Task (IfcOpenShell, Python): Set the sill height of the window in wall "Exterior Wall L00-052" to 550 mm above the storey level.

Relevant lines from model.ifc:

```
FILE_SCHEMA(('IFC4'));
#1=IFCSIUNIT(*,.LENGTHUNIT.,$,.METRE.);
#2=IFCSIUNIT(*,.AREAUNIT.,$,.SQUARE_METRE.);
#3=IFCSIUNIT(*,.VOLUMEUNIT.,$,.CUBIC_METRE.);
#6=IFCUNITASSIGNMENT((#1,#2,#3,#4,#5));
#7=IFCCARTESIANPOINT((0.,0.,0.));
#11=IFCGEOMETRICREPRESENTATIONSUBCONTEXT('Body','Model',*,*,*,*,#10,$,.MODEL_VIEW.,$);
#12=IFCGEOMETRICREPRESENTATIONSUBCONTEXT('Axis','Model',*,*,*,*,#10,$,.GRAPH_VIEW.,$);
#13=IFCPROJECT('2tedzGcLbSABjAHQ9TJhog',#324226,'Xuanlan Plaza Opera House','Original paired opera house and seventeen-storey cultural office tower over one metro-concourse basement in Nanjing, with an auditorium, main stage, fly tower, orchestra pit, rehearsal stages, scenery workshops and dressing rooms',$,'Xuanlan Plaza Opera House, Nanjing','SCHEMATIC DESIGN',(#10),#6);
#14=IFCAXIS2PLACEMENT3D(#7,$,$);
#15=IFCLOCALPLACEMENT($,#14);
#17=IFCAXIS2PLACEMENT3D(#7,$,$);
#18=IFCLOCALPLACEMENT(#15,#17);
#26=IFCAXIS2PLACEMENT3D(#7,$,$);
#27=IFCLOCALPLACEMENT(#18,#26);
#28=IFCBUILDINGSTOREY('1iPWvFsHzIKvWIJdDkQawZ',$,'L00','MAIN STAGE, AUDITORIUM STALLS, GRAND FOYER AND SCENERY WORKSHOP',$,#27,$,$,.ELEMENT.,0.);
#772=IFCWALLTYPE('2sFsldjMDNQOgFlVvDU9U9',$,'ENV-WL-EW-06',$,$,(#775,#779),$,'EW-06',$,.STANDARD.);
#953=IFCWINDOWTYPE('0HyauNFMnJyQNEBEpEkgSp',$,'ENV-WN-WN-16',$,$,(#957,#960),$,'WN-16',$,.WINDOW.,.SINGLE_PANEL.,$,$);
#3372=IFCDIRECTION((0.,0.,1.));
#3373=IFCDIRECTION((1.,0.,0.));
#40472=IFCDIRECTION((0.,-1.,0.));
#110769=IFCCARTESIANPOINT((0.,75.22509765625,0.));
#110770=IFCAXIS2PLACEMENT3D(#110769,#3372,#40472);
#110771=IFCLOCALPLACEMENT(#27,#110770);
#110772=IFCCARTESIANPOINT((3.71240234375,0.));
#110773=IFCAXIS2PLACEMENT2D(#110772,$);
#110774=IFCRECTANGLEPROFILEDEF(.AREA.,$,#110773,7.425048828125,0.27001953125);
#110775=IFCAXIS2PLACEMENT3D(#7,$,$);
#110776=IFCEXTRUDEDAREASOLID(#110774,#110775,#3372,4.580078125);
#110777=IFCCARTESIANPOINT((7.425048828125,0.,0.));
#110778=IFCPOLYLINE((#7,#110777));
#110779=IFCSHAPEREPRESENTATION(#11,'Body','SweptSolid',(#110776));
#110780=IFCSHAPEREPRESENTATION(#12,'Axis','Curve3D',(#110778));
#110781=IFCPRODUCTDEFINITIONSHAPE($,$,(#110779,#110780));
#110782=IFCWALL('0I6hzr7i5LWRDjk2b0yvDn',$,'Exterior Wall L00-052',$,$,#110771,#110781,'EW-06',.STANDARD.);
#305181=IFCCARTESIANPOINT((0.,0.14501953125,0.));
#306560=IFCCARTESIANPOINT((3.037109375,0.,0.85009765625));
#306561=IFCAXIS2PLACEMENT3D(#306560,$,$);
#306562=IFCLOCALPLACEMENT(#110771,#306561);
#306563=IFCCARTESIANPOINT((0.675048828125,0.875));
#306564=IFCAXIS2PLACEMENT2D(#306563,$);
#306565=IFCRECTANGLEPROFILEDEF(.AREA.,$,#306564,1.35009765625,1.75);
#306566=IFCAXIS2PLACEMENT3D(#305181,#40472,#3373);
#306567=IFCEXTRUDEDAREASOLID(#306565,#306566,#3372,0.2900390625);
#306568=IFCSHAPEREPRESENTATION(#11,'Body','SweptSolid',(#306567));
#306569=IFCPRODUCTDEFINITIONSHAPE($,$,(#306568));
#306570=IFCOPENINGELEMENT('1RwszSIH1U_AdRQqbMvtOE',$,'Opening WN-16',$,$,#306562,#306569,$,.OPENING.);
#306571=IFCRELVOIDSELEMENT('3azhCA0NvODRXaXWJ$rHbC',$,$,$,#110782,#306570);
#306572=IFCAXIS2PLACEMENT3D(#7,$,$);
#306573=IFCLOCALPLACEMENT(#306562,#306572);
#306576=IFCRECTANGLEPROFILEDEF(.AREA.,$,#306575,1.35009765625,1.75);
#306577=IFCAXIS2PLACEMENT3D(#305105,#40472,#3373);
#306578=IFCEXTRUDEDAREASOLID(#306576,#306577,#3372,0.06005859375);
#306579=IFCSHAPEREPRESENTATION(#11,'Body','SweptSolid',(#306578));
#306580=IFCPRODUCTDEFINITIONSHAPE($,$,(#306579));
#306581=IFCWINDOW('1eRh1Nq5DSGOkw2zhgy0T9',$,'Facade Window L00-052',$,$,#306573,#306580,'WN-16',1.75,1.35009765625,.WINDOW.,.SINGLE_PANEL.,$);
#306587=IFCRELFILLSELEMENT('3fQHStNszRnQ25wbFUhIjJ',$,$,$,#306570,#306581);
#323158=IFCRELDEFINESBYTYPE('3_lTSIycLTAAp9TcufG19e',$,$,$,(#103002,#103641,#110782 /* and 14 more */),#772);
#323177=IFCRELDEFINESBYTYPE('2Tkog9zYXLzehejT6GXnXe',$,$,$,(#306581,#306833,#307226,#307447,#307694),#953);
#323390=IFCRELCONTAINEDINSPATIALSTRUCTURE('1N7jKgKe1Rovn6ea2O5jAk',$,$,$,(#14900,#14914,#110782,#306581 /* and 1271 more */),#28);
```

```python
import numpy as np
import ifcopenshell
import ifcopenshell.api.geometry
import ifcopenshell.geom
import ifcopenshell.util.element
import ifcopenshell.util.placement
import ifcopenshell.util.shape
import ifcopenshell.util.unit

model = ifcopenshell.open("model.ifc")
unit_scale = ifcopenshell.util.unit.calculate_unit_scale(model)

window = model.by_guid("1eRh1Nq5DSGOkw2zhgy0T9")
opening = window.FillsVoids[0].RelatingOpeningElement
storey = ifcopenshell.util.element.get_container(window, ifc_class="IfcBuildingStorey")
level = ifcopenshell.util.placement.get_local_placement(storey.ObjectPlacement)[2, 3]

# The opening's origin need not be at the sill, so measure its lowest point.
shape = ifcopenshell.geom.create_shape(ifcopenshell.geom.settings(), opening)
bottom = ifcopenshell.util.shape.get_shape_bottom_elevation(shape, shape.geometry) / unit_scale
dz = level + 0.55 - bottom

shift = np.array([0.0, 0.0, dz])
# The window is placed relative to its opening, so it follows when the opening moves.
matrix = ifcopenshell.util.placement.get_local_placement(opening.ObjectPlacement)
matrix[:3, 3] += shift
ifcopenshell.api.geometry.edit_object_placement(
    model, product=opening, matrix=matrix, is_si=False, should_transform_children=True
)

print(f"moved by {dz * unit_scale:+.3f} m")

model.write("model-out.ifc")
```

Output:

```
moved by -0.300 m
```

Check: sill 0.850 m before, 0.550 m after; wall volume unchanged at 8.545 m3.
